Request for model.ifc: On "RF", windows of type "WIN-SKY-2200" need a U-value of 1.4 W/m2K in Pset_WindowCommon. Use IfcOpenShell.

First a look at what the model holds.

```python
import ifcopenshell
import ifcopenshell.util.element

model = ifcopenshell.open("model.ifc")
print(model.schema)
storey = next(s for s in model.by_type("IfcBuildingStorey") if s.Name == "RF")
windows = [e for e in ifcopenshell.util.element.get_decomposition(storey) if e.is_a("IfcWindow")]
seen = {}
for e in windows:
    element_type = ifcopenshell.util.element.get_type(e)
    key = (element_type.Name if element_type != e and element_type else None, ifcopenshell.util.element.get_pset(e, "Pset_WindowCommon", "ThermalTransmittance"))
    seen[key] = seen.get(key, 0) + 1
for (name, value), count in sorted(seen.items(), key=str):
    print(count, "x", name, "|", value)
```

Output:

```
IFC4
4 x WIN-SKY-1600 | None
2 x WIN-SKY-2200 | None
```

```python
import ifcopenshell
import ifcopenshell.api.pset
import ifcopenshell.util.element

model = ifcopenshell.open("model.ifc")

storey = next(s for s in model.by_type("IfcBuildingStorey") if s.Name == "RF")
windows = [e for e in ifcopenshell.util.element.get_decomposition(storey) if e.is_a("IfcWindow")]

count = 0
for e in windows:
    element_type = ifcopenshell.util.element.get_type(e)
    if element_type in (None, e) or element_type.Name != "WIN-SKY-2200":
        continue
    found = ifcopenshell.util.element.get_pset(e, "Pset_WindowCommon", should_inherit=False)
    if found:
        pset = model.by_id(found["id"])
        if len(ifcopenshell.util.element.get_elements_by_pset(pset)) > 1:
            pset = ifcopenshell.api.pset.unshare_pset(model, products=[e], pset=pset)[0]
    else:
        pset = ifcopenshell.api.pset.add_pset(model, product=e, name="Pset_WindowCommon")
    ifcopenshell.api.pset.edit_pset(model, pset=pset, properties={"ThermalTransmittance": 1.4})
    count += 1

print(count, "windows updated")

model.write("model_edited.ifc")
```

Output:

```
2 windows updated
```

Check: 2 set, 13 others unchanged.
